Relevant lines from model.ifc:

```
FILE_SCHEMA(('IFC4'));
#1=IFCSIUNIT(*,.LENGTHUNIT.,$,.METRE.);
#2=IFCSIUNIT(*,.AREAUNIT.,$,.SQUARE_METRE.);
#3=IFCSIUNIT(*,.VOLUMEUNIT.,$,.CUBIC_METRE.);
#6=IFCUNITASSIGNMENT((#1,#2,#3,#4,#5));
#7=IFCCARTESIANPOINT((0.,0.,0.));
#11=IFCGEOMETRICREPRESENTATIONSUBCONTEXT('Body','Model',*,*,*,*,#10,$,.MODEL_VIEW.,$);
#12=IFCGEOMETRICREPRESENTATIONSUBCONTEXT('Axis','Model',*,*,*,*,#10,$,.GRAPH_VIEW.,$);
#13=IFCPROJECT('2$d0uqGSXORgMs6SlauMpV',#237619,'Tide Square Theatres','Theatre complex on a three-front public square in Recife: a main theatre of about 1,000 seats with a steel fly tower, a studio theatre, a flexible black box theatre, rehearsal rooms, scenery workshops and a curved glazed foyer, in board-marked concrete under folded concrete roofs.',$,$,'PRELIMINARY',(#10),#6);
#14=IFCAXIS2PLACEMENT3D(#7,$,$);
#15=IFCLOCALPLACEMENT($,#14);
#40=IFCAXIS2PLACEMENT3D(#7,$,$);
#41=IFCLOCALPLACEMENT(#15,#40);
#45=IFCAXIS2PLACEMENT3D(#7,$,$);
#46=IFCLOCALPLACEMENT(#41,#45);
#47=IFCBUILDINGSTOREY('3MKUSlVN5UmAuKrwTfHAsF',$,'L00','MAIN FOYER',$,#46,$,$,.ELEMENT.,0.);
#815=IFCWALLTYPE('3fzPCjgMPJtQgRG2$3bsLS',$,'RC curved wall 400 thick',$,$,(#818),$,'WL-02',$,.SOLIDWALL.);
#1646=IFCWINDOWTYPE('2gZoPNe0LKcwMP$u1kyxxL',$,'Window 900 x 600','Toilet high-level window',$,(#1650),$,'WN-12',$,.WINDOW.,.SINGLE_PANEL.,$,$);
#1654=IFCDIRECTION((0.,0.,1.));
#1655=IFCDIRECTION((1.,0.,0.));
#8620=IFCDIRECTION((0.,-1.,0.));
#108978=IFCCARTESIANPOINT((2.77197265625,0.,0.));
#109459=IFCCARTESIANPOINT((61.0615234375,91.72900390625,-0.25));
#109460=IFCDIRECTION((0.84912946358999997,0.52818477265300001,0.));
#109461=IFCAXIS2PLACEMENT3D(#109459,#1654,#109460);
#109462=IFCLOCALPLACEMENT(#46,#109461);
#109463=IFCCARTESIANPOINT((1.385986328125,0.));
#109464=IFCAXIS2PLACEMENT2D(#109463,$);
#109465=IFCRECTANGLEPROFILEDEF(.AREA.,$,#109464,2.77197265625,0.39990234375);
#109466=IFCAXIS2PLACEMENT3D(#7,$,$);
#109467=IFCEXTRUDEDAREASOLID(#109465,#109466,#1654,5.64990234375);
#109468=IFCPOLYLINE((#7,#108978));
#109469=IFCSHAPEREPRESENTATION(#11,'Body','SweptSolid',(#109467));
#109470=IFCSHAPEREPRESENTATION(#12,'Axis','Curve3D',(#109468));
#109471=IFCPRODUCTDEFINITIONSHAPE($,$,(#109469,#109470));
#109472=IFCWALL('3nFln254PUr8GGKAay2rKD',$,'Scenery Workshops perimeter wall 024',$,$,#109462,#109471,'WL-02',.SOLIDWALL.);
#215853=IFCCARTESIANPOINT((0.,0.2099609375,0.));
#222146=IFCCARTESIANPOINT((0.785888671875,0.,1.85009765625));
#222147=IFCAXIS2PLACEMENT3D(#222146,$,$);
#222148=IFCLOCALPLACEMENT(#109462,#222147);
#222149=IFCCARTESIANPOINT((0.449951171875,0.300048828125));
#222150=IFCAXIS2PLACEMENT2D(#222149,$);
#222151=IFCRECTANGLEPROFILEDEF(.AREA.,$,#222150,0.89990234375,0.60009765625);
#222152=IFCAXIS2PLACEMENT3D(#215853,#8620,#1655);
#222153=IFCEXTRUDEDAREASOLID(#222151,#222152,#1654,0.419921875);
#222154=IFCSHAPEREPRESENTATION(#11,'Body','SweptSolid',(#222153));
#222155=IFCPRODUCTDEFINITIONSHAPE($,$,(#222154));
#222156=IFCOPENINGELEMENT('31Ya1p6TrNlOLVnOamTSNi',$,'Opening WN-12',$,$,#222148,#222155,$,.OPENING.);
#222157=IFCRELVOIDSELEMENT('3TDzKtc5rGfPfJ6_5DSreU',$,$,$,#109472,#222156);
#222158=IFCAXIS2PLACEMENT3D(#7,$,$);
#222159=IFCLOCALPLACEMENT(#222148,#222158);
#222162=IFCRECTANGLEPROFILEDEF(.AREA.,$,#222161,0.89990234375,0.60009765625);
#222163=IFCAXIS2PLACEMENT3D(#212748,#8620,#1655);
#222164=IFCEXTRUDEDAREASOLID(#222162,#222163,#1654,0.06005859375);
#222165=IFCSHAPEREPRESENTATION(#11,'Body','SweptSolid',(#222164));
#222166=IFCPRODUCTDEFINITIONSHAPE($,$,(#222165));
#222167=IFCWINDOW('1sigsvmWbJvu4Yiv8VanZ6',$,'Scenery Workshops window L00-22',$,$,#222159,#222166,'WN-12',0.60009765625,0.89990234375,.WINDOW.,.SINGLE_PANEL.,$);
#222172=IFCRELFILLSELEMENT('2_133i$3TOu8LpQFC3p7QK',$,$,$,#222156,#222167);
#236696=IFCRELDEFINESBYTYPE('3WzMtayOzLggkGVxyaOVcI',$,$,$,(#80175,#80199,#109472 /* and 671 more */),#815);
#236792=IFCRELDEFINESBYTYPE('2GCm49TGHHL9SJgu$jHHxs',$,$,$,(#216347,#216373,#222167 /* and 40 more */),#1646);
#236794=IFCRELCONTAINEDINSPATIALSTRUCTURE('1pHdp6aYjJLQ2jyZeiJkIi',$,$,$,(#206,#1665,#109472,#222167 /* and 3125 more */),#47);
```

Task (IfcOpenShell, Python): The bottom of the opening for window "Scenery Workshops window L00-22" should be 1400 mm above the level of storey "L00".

```python
import numpy as np
import ifcopenshell
import ifcopenshell.api.geometry
import ifcopenshell.geom
import ifcopenshell.util.element
import ifcopenshell.util.placement
import ifcopenshell.util.shape
import ifcopenshell.util.unit

model = ifcopenshell.open("model.ifc")
unit_scale = ifcopenshell.util.unit.calculate_unit_scale(model)

window = model.by_guid("1sigsvmWbJvu4Yiv8VanZ6")
opening = window.FillsVoids[0].RelatingOpeningElement
storey = ifcopenshell.util.element.get_container(window, ifc_class="IfcBuildingStorey")
level = ifcopenshell.util.placement.get_local_placement(storey.ObjectPlacement)[2, 3]

# The opening's origin need not be at the sill, so measure its lowest point.
shape = ifcopenshell.geom.create_shape(ifcopenshell.geom.settings(), opening)
bottom = ifcopenshell.util.shape.get_shape_bottom_elevation(shape, shape.geometry) / unit_scale
dz = level + 1.4 - bottom

shift = np.array([0.0, 0.0, dz])
# The window is placed relative to its opening, so it follows when the opening moves.
matrix = ifcopenshell.util.placement.get_local_placement(opening.ObjectPlacement)
matrix[:3, 3] += shift
ifcopenshell.api.geometry.edit_object_placement(
    model, product=opening, matrix=matrix, is_si=False, should_transform_children=True
)

print(f"moved by {dz * unit_scale:+.3f} m")

model.write("model_updated.ifc")
```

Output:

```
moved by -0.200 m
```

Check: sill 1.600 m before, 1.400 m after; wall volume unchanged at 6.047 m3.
